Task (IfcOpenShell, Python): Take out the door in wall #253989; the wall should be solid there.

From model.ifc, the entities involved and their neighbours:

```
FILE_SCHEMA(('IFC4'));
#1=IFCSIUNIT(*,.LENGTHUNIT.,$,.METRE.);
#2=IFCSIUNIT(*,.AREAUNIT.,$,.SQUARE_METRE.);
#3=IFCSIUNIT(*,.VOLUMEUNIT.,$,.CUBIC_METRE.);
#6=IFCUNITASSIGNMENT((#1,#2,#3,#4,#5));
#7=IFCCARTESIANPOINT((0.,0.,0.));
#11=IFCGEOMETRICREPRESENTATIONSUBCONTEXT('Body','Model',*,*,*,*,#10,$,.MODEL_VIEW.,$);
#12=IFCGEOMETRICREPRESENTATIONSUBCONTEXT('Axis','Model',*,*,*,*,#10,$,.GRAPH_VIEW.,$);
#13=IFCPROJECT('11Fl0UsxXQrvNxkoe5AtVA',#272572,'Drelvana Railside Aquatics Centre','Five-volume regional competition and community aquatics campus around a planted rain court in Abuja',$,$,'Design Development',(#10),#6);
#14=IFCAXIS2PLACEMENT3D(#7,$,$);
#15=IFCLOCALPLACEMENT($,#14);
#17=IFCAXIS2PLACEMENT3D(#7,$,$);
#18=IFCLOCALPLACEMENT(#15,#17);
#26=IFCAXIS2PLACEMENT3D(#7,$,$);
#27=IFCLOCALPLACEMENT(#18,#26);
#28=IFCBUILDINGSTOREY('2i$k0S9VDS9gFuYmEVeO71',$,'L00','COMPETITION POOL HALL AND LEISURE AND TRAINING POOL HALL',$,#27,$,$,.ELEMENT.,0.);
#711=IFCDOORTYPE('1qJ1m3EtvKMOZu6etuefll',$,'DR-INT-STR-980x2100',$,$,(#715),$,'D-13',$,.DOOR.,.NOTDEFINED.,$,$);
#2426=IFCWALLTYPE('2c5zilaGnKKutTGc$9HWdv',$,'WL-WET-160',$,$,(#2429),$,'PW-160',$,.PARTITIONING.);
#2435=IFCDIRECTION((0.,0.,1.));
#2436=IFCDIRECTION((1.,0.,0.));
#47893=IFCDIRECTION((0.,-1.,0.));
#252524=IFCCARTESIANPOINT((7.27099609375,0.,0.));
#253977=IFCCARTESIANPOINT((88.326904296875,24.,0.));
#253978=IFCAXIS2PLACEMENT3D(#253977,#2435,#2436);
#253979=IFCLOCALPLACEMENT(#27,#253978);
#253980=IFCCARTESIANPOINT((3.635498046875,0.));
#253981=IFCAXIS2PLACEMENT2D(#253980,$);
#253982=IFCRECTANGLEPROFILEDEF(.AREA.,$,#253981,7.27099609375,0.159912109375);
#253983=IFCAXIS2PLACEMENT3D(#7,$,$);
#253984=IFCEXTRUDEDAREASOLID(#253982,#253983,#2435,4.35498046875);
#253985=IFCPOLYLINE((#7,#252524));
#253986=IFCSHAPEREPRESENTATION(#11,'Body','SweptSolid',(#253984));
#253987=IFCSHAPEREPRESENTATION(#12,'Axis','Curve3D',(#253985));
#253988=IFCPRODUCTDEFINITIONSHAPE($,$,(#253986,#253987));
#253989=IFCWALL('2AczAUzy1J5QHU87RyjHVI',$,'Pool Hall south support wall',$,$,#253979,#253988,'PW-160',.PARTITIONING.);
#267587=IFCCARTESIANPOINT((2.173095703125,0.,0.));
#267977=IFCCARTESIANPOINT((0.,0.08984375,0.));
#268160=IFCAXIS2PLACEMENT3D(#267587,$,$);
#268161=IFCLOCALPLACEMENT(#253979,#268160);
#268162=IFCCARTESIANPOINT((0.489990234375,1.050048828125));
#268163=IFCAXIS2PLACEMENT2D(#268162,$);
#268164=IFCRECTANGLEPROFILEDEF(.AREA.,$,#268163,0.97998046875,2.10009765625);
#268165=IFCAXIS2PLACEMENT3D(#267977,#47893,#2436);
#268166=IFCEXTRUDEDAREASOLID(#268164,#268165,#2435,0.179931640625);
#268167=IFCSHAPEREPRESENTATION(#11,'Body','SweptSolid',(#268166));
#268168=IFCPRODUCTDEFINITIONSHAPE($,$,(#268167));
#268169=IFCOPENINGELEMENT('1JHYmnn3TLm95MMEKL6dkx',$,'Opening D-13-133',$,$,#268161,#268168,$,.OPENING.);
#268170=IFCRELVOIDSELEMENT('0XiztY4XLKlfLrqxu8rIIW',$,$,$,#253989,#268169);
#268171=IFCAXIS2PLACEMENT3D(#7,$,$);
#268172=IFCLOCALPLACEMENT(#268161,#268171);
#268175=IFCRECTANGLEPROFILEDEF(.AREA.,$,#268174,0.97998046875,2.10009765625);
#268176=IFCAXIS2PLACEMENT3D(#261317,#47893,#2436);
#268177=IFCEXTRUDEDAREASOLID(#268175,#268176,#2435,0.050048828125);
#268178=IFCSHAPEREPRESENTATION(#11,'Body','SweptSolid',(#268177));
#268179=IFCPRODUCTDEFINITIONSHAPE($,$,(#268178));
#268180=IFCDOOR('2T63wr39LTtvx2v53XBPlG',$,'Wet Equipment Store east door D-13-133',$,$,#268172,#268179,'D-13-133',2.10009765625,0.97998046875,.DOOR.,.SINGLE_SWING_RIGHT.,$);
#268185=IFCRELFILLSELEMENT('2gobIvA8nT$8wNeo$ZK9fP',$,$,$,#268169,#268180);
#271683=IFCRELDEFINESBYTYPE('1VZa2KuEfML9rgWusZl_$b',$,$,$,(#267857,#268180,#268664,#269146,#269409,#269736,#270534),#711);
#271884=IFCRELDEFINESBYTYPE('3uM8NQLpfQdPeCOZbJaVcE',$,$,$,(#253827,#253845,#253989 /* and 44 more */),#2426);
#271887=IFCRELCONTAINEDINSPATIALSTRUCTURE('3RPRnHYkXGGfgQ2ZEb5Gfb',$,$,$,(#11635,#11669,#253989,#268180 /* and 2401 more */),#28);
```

```python
import ifcopenshell
import ifcopenshell.api.feature
import ifcopenshell.api.root
import ifcopenshell.geom
import ifcopenshell.util.shape

model = ifcopenshell.open("model.ifc")
settings = ifcopenshell.geom.settings()


def volume(element):
    """Net volume in cubic metres, openings subtracted."""
    shape = ifcopenshell.geom.create_shape(settings, element)
    return ifcopenshell.util.shape.get_volume(shape.geometry)


door = model.by_guid("2T63wr39LTtvx2v53XBPlG")
opening = door.FillsVoids[0].RelatingOpeningElement
wall = opening.VoidsElements[0].RelatingBuildingElement
before = volume(wall)

ifcopenshell.api.root.remove_product(model, product=door)
ifcopenshell.api.feature.remove_feature(model, feature=opening)

after = volume(wall)

print(f"wall volume {before:.3f} -> {after:.3f} m3")

model.write("model-out.ifc")
```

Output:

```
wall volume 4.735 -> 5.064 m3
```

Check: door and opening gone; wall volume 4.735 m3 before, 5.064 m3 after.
